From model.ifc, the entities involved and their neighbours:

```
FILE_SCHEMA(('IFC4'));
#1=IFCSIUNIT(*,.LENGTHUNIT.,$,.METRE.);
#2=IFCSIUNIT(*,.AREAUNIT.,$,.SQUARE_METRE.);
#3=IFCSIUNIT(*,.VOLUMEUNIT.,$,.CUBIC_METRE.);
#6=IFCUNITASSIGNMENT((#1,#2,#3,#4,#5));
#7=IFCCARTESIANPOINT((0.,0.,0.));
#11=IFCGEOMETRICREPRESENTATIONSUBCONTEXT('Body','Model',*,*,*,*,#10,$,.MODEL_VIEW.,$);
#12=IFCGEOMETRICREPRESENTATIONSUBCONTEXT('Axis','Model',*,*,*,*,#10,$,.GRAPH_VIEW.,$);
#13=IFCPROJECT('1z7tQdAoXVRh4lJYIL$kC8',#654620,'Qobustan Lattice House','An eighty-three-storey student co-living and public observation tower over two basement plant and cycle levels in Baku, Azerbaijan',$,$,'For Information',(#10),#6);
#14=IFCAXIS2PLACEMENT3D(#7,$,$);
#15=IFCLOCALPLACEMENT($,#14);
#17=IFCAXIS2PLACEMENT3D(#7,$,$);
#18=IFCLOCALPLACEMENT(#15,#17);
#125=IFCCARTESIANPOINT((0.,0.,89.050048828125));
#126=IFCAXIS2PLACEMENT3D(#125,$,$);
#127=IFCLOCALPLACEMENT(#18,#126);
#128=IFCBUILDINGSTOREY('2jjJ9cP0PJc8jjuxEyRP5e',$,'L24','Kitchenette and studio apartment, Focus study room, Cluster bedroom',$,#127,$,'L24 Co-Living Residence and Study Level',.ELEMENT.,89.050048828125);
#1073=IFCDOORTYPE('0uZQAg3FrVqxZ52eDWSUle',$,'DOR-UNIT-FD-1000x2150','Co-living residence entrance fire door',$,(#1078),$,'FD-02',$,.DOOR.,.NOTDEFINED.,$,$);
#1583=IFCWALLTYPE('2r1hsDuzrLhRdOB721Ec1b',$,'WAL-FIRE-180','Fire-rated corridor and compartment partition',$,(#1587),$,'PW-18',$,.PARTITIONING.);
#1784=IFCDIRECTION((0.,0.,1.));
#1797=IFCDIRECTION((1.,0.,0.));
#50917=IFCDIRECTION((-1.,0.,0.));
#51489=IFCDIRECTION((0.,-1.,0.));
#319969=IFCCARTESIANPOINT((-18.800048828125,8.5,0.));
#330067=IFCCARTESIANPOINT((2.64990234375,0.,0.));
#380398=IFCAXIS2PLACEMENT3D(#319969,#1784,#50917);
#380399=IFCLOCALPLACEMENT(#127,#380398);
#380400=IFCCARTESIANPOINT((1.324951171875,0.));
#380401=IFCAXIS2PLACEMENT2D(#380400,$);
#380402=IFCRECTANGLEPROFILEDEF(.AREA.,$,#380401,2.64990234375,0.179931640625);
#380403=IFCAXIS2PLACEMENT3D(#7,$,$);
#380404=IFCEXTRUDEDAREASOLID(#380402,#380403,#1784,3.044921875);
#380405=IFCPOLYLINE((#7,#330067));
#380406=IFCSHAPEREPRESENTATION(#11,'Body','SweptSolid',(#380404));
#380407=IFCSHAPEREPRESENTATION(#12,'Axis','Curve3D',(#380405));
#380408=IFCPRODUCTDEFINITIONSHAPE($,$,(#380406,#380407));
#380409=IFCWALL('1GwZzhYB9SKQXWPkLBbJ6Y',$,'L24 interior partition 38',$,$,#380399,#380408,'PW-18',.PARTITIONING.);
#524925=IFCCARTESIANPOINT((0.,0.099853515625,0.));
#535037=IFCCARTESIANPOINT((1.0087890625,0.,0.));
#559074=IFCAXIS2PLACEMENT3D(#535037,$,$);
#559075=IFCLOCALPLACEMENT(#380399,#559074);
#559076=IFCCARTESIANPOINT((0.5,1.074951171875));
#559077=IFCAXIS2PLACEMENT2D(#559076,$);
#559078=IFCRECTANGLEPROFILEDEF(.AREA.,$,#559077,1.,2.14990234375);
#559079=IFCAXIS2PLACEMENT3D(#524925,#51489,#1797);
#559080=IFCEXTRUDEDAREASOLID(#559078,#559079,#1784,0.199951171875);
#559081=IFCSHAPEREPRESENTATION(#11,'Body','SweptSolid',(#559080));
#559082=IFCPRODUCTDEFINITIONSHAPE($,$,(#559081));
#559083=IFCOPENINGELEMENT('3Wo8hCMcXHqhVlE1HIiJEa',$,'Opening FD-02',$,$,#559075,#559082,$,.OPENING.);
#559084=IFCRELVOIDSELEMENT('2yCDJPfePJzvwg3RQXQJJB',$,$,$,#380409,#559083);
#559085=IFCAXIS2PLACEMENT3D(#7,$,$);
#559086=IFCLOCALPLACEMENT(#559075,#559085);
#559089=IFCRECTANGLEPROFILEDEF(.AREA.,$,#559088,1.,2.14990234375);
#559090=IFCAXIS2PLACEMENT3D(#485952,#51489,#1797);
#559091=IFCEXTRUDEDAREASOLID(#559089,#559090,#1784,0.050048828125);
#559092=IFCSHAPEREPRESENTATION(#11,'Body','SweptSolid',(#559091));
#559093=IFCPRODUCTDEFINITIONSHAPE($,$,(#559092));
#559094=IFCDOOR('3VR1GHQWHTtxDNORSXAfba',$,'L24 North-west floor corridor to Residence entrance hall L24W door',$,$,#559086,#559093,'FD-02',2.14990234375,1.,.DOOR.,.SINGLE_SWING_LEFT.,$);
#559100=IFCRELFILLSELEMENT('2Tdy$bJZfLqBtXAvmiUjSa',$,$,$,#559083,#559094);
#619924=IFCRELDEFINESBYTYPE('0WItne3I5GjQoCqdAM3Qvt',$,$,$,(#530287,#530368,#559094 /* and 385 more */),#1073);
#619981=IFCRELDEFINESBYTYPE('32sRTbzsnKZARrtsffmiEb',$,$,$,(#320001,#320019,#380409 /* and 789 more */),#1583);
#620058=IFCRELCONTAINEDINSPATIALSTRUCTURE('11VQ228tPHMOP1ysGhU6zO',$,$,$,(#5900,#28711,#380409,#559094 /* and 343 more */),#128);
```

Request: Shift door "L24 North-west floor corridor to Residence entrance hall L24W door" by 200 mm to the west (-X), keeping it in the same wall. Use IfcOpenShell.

```python
import ifcopenshell
import ifcopenshell.api.geometry
import ifcopenshell.util.placement

model = ifcopenshell.open("model.ifc")

door = model.by_guid("3VR1GHQWHTtxDNORSXAfba")
opening = door.FillsVoids[0].RelatingOpeningElement
wall = opening.VoidsElements[0].RelatingBuildingElement

wall_matrix = ifcopenshell.util.placement.get_local_placement(wall.ObjectPlacement)
shift = wall_matrix[:3, 0] * 0.2
before = ifcopenshell.util.placement.get_local_placement(door.ObjectPlacement)[:3, 3].copy()

# The door is placed relative to its opening, so it follows when the opening moves.
matrix = ifcopenshell.util.placement.get_local_placement(opening.ObjectPlacement)
matrix[:3, 3] += shift
ifcopenshell.api.geometry.edit_object_placement(
    model, product=opening, matrix=matrix, is_si=False, should_transform_children=True
)

after = ifcopenshell.util.placement.get_local_placement(door.ObjectPlacement)[:3, 3]
print("door moved by", (after - before).round(3) + 0.0)

model.write("model_edited.ifc")
```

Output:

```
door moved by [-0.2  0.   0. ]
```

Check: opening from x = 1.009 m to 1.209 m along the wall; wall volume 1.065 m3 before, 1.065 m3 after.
